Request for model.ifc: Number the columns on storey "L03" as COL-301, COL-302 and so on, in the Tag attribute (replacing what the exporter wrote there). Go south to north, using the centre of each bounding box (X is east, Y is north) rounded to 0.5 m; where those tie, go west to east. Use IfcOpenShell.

First a look at what the model holds.

```python
import ifcopenshell
import ifcopenshell.util.element
import ifcopenshell.util.placement

model = ifcopenshell.open("model.ifc")
print(model.schema)
storey = next(s for s in model.by_type("IfcBuildingStorey") if s.Name == "L03")
columns = [e for e in ifcopenshell.util.element.get_decomposition(storey) if e.is_a("IfcColumn")]
for e in sorted(columns, key=lambda e: e.id()):
    origin = ifcopenshell.util.placement.get_local_placement(e.ObjectPlacement)[:3, 3]
    print(e.id(), e.Tag, e.Name, origin.round(2) + 0.0, sep=" | ")
```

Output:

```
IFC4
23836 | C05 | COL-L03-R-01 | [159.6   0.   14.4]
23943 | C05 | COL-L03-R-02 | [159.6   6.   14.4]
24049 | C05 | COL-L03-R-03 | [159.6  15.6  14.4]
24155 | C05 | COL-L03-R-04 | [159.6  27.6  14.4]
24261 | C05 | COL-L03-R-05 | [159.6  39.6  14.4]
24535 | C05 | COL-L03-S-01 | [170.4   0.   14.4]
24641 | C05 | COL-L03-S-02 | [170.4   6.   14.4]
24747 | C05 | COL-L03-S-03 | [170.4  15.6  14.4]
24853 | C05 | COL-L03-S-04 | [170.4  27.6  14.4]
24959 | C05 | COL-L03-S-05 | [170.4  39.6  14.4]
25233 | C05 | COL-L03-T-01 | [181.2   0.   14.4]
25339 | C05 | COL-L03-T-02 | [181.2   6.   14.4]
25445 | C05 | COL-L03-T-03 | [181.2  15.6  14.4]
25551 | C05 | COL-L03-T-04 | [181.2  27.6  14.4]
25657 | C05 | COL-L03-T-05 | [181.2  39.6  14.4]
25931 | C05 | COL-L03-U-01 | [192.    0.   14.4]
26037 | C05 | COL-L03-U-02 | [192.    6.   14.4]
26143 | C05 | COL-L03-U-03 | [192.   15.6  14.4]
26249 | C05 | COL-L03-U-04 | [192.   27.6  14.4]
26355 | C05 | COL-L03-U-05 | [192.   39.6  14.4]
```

```python
import ifcopenshell
import ifcopenshell.geom
import ifcopenshell.util.element
import ifcopenshell.util.shape

model = ifcopenshell.open("model.ifc")
settings = ifcopenshell.geom.settings()
settings.set("use-world-coords", True)


def centre(element):
    shape = ifcopenshell.geom.create_shape(settings, element)
    return ifcopenshell.util.shape.get_bbox_centroid(shape.geometry)


storey = next(s for s in model.by_type("IfcBuildingStorey") if s.Name == "L03")
columns = [e for e in ifcopenshell.util.element.get_decomposition(storey) if e.is_a("IfcColumn")]

# Insertion points can sit at a corner or the storey origin, so sort by the geometry (in metres).
centres = {e: centre(e) for e in columns}
columns.sort(key=lambda e: (round(centres[e][1] / 0.5), centres[e][0]))

for i, e in enumerate(columns, start=1):
    number = f"COL-3{i:02d}"
    e.Tag = number
    print(e.id(), number)

model.write("model_rev.ifc")
```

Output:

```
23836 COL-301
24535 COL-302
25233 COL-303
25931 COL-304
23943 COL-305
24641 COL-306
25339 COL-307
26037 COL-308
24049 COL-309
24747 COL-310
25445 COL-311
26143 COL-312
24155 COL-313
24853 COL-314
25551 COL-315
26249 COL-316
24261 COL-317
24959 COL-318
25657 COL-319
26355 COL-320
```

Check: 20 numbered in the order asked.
